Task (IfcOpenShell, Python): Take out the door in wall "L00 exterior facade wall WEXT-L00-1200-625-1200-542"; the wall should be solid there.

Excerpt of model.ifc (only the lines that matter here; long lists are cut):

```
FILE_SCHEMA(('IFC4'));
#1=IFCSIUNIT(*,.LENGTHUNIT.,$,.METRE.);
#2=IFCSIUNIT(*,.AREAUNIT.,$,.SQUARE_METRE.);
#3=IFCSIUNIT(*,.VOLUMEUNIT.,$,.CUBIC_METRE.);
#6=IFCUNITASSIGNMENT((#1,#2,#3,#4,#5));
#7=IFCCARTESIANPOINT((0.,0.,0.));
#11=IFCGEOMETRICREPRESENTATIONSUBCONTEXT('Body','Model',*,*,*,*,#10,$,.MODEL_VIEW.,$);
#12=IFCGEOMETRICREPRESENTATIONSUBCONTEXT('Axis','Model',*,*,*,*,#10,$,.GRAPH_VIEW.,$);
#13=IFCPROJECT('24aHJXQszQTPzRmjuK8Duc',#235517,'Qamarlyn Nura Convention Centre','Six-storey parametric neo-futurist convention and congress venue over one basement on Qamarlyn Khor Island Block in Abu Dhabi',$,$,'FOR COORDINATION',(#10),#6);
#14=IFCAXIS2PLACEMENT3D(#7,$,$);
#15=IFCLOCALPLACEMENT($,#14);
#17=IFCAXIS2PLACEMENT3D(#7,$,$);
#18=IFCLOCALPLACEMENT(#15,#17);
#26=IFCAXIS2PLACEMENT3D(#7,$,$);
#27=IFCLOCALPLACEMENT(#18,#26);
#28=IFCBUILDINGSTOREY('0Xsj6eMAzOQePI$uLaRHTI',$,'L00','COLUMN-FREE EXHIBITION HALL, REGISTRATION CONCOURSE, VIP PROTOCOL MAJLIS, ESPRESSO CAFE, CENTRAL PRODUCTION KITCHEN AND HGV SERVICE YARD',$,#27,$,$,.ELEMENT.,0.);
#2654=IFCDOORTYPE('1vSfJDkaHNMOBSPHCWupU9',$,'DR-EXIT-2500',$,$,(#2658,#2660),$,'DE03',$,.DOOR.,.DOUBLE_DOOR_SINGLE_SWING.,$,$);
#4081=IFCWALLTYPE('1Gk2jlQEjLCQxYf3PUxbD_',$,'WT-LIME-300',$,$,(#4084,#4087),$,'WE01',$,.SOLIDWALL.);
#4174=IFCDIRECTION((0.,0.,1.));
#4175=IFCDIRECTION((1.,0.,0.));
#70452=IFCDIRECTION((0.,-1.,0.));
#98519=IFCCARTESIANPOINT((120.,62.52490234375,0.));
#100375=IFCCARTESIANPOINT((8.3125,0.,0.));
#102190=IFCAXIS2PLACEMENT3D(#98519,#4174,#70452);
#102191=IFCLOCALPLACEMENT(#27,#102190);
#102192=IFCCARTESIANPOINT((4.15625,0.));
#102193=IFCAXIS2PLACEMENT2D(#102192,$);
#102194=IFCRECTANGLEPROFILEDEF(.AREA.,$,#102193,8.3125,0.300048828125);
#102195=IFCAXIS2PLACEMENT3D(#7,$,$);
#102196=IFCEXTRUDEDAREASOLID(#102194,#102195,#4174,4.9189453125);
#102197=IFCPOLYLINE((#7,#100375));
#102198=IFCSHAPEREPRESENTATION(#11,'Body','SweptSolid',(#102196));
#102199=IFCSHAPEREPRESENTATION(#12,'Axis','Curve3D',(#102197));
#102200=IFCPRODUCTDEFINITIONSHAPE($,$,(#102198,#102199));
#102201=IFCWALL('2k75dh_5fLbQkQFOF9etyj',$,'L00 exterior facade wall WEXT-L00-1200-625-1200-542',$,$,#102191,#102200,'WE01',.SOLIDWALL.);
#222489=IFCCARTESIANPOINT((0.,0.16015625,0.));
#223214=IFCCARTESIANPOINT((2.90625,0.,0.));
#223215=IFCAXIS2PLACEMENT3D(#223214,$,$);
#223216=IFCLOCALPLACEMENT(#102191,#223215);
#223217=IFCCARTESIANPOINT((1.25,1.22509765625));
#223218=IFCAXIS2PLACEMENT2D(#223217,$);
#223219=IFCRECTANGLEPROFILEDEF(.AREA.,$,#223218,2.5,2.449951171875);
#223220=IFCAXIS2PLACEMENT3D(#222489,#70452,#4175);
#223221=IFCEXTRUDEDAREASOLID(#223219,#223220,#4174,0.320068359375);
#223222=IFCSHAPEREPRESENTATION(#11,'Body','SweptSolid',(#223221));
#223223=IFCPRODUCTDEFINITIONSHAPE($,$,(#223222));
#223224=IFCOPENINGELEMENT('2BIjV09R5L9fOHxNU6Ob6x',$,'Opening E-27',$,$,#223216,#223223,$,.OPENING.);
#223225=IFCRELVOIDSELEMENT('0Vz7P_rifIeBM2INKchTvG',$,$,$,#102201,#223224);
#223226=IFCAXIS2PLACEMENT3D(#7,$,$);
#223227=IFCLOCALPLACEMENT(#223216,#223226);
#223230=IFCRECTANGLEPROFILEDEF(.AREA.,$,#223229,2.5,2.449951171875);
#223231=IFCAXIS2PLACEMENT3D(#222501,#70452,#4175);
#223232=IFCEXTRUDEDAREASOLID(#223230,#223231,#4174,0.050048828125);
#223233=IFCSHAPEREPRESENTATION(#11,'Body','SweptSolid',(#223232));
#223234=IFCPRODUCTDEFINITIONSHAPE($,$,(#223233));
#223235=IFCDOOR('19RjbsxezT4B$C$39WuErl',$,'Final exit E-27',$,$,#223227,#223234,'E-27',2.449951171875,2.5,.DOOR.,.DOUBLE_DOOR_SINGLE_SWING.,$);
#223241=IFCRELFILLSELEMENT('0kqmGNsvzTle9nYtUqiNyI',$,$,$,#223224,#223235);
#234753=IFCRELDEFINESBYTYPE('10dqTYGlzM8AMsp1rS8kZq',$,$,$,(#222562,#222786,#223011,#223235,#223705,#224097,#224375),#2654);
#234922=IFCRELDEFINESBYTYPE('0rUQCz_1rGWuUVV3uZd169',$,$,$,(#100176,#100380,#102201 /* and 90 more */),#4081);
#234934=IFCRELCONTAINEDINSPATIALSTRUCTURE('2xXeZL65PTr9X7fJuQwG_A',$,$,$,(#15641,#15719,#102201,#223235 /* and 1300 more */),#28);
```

```python
import ifcopenshell
import ifcopenshell.api.feature
import ifcopenshell.api.root
import ifcopenshell.geom
import ifcopenshell.util.shape

model = ifcopenshell.open("model.ifc")
settings = ifcopenshell.geom.settings()


def volume(element):
    """Net volume in cubic metres, openings subtracted."""
    shape = ifcopenshell.geom.create_shape(settings, element)
    return ifcopenshell.util.shape.get_volume(shape.geometry)


door = model.by_id(223235)
opening = door.FillsVoids[0].RelatingOpeningElement
wall = opening.VoidsElements[0].RelatingBuildingElement
before = volume(wall)

ifcopenshell.api.root.remove_product(model, product=door)
ifcopenshell.api.feature.remove_feature(model, feature=opening)

after = volume(wall)

print(f"wall volume {before:.3f} -> {after:.3f} m3")

model.write("model_rev.ifc")
```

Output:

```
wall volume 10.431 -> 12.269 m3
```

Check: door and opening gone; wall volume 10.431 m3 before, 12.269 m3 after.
